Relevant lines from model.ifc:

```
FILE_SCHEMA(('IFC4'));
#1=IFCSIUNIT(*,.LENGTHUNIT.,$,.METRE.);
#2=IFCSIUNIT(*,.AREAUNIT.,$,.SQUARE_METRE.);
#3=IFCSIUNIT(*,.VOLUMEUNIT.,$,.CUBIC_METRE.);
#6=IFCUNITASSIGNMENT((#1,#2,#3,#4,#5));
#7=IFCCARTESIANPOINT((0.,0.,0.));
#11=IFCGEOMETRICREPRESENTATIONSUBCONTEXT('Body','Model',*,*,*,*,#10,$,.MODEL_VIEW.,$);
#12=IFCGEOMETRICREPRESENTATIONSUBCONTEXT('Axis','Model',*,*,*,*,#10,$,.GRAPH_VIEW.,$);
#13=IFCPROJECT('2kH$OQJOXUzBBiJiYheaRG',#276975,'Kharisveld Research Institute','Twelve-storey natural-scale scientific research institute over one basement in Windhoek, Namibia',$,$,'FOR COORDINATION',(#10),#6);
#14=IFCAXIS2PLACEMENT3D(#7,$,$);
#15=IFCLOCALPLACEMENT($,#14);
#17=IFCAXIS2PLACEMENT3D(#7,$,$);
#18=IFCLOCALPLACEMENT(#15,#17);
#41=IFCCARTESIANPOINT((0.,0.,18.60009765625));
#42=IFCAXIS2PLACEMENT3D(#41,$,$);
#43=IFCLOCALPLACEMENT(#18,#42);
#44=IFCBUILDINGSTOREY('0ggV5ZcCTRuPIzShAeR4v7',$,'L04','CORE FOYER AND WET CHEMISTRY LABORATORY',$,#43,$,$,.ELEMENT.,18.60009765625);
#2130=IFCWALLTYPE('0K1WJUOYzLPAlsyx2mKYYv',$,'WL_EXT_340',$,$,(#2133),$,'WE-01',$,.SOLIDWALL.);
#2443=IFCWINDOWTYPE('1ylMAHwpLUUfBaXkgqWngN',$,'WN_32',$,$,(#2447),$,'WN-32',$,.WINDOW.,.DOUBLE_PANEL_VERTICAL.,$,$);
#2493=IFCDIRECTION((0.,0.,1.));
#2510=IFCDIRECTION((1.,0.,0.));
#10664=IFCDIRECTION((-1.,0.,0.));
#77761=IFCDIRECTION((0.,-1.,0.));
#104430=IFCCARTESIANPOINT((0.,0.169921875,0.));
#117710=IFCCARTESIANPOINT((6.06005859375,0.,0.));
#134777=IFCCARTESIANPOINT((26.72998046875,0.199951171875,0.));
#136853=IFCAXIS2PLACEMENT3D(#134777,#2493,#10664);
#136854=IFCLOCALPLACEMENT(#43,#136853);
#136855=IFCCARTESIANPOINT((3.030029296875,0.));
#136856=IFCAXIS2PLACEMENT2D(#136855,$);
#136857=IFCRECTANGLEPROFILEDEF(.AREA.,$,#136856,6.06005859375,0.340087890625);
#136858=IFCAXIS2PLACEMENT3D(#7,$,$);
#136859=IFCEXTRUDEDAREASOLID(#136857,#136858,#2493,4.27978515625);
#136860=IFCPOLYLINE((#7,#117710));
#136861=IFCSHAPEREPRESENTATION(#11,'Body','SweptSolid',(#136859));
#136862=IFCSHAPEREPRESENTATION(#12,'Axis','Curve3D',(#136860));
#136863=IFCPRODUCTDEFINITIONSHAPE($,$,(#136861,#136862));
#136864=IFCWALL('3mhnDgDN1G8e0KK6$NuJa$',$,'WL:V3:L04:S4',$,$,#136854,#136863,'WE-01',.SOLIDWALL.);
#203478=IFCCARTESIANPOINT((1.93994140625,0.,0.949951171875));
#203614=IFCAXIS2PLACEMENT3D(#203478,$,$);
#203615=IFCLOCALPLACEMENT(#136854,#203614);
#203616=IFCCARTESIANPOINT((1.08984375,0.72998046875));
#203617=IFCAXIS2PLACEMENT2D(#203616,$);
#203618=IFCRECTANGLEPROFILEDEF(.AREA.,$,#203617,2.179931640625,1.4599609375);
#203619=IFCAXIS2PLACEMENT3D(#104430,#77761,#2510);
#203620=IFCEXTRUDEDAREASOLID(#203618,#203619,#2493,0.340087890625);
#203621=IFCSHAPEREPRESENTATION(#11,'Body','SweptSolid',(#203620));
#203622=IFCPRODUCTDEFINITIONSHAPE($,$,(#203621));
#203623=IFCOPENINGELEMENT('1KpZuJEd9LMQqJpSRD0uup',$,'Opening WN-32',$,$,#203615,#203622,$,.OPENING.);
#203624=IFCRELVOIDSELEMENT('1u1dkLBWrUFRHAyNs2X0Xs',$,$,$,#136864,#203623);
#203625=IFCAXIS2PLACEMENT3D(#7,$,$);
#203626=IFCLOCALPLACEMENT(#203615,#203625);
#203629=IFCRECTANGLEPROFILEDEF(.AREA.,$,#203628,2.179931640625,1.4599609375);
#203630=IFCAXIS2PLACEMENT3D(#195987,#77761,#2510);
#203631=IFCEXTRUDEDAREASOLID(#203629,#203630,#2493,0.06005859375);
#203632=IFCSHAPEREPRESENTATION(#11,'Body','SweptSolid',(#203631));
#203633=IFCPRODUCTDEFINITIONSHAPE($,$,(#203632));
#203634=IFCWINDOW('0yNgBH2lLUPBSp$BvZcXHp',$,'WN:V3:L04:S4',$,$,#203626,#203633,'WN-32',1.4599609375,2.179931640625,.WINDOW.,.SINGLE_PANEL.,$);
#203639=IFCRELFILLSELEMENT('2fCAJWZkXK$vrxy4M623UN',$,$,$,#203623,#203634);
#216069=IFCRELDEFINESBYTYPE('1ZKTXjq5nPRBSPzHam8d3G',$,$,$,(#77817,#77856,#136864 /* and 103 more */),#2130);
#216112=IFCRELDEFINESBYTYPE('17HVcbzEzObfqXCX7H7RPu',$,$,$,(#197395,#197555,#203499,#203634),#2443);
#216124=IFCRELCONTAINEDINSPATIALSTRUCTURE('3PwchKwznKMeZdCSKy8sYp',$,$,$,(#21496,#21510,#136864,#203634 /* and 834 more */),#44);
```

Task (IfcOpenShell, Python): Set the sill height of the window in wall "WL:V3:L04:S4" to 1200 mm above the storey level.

```python
import numpy as np
import ifcopenshell
import ifcopenshell.api.geometry
import ifcopenshell.geom
import ifcopenshell.util.element
import ifcopenshell.util.placement
import ifcopenshell.util.shape
import ifcopenshell.util.unit

model = ifcopenshell.open("model.ifc")
unit_scale = ifcopenshell.util.unit.calculate_unit_scale(model)

window = model.by_id(203634)
opening = window.FillsVoids[0].RelatingOpeningElement
storey = ifcopenshell.util.element.get_container(window, ifc_class="IfcBuildingStorey")
level = ifcopenshell.util.placement.get_local_placement(storey.ObjectPlacement)[2, 3]

# The opening's origin need not be at the sill, so measure its lowest point.
shape = ifcopenshell.geom.create_shape(ifcopenshell.geom.settings(), opening)
bottom = ifcopenshell.util.shape.get_shape_bottom_elevation(shape, shape.geometry) / unit_scale
dz = level + 1.2 / unit_scale - bottom

shift = np.array([0.0, 0.0, dz])
# The window is placed relative to its opening, so it follows when the opening moves.
matrix = ifcopenshell.util.placement.get_local_placement(opening.ObjectPlacement)
matrix[:3, 3] += shift
ifcopenshell.api.geometry.edit_object_placement(
    model, product=opening, matrix=matrix, is_si=False, should_transform_children=True
)

print(f"moved by {dz * unit_scale:+.3f} m")

model.write("model_updated.ifc")
```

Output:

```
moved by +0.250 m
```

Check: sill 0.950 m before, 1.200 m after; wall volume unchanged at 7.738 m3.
